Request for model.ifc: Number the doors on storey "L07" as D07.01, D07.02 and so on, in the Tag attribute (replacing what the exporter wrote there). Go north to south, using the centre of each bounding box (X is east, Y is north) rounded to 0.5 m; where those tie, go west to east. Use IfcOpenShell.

First a look at what the model holds.

```python
import ifcopenshell
import ifcopenshell.util.element
import ifcopenshell.util.placement

model = ifcopenshell.open("model.ifc")
print(model.schema)
storey = next(s for s in model.by_type("IfcBuildingStorey") if s.Name == "L07")
doors = [e for e in ifcopenshell.util.element.get_decomposition(storey) if e.is_a("IfcDoor")]
for e in sorted(doors, key=lambda e: e.id()):
    origin = ifcopenshell.util.placement.get_local_placement(e.ObjectPlacement)[:3, 3]
    print(e.id(), e.Tag, e.Name, origin.round(2) + 0.0, sep=" | ")
```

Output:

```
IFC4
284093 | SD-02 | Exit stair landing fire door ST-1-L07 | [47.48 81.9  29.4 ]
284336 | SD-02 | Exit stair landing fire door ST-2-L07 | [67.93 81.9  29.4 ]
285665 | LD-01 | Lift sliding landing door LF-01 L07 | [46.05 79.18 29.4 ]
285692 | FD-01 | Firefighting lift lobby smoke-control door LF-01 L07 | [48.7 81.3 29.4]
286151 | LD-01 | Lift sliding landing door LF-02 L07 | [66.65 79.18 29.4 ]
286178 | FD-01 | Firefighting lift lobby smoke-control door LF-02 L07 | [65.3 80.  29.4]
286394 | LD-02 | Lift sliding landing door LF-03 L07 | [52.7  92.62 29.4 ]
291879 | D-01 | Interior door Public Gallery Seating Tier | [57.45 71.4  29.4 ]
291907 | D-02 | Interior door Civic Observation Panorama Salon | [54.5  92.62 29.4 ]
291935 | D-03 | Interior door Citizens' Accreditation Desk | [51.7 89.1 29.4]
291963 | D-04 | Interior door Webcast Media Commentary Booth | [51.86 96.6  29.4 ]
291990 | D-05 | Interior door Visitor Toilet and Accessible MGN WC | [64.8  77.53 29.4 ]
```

```python
import ifcopenshell
import ifcopenshell.geom
import ifcopenshell.util.element
import ifcopenshell.util.shape

model = ifcopenshell.open("model.ifc")
settings = ifcopenshell.geom.settings()
settings.set("use-world-coords", True)


def centre(element):
    shape = ifcopenshell.geom.create_shape(settings, element)
    return ifcopenshell.util.shape.get_bbox_centroid(shape.geometry)


storey = next(s for s in model.by_type("IfcBuildingStorey") if s.Name == "L07")
doors = [e for e in ifcopenshell.util.element.get_decomposition(storey) if e.is_a("IfcDoor")]

# Insertion points can sit at a corner or the storey origin, so sort by the geometry (in metres).
centres = {e: centre(e) for e in doors}
doors.sort(key=lambda e: (-round(centres[e][1] / 0.5), centres[e][0]))

for i, e in enumerate(doors, start=1):
    number = f"D07.{i:02d}"
    e.Tag = number
    print(e.id(), number)

model.write("model-out.ifc")
```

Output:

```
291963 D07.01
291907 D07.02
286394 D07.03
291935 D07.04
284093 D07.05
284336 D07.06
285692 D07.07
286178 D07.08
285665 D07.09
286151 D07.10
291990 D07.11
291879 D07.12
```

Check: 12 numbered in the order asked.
